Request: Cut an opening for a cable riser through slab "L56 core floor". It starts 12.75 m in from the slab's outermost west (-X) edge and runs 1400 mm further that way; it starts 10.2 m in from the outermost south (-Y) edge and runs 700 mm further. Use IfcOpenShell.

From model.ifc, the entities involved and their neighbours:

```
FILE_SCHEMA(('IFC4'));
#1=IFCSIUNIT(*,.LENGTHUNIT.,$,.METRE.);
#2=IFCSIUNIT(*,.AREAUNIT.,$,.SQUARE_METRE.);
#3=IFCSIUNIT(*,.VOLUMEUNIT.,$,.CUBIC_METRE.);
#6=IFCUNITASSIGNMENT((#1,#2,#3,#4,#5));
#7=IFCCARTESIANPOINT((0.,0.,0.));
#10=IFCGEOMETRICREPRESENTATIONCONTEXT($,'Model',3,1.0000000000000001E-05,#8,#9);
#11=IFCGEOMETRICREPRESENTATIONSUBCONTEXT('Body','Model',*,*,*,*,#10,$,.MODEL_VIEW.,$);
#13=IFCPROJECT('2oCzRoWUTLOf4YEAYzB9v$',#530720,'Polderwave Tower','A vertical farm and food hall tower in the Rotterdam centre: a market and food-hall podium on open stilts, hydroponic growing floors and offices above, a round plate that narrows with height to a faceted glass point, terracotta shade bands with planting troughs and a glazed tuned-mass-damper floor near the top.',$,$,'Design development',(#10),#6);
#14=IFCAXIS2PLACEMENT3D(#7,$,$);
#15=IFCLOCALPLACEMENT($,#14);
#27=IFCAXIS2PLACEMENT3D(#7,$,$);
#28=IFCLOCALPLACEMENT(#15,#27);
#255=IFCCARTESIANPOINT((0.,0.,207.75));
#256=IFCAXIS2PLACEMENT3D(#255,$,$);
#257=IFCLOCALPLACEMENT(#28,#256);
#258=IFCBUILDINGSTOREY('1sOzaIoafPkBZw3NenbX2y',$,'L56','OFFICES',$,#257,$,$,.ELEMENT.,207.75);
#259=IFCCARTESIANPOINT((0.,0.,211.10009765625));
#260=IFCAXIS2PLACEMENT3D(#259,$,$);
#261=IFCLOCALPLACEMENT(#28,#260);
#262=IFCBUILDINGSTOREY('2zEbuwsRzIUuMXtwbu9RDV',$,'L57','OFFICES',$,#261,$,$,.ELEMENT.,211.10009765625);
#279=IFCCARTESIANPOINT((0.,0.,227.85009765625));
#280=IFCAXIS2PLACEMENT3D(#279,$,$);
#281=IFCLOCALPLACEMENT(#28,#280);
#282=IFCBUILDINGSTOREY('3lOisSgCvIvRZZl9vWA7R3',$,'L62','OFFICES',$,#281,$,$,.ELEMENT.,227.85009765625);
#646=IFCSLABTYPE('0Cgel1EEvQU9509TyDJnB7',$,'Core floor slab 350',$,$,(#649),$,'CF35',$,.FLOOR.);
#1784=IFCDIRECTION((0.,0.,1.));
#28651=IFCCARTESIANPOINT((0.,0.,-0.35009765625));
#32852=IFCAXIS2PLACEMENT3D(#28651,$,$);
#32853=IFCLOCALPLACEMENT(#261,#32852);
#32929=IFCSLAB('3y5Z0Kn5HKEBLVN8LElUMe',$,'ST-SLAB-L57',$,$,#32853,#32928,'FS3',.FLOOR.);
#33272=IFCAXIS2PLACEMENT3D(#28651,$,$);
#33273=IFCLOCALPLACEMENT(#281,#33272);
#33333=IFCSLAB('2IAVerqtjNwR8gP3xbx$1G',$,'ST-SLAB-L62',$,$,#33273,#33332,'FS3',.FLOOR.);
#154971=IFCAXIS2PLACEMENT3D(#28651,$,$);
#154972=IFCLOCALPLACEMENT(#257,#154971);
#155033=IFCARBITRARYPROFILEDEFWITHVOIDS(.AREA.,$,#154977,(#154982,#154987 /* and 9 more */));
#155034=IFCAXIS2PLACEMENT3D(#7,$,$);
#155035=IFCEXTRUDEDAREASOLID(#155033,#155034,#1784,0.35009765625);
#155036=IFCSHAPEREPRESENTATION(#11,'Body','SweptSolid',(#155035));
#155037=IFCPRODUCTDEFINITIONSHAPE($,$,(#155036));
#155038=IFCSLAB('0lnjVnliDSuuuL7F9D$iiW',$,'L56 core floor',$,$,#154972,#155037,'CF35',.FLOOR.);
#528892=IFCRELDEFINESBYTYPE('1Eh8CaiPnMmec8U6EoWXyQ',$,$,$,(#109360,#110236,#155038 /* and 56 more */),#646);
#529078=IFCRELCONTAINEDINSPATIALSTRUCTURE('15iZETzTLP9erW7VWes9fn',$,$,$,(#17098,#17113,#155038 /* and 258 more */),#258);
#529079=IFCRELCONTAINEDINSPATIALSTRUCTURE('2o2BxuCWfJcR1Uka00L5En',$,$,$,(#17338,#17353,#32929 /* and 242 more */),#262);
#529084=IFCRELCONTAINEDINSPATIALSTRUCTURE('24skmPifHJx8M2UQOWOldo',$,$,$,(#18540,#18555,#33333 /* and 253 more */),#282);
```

```python
import numpy as np
import ifcopenshell
import ifcopenshell.api.feature
import ifcopenshell.api.geometry
import ifcopenshell.api.root
import ifcopenshell.geom
import ifcopenshell.util.placement
import ifcopenshell.util.representation
import ifcopenshell.util.shape
import ifcopenshell.util.unit

model = ifcopenshell.open("model.ifc")
unit_scale = ifcopenshell.util.unit.calculate_unit_scale(model)
settings = ifcopenshell.geom.settings()


def volume(element):
    """Net volume in cubic metres, openings subtracted."""
    shape = ifcopenshell.geom.create_shape(settings, element)
    return ifcopenshell.util.shape.get_volume(shape.geometry)


slab = model.by_guid("0lnjVnliDSuuuL7F9D$iiW")
before = volume(slab)

# Extent in the slab's own axes, in metres. The edges named are its -X and -Y sides.
slab_shape = ifcopenshell.geom.create_shape(settings, slab)
vertices = ifcopenshell.util.shape.get_vertices(slab_shape.geometry)
x_min, y_min, bottom = vertices.min(axis=0)
top = vertices[:, 2].max()

opening = ifcopenshell.api.root.create_entity(model, ifc_class="IfcOpeningElement", name="Cable riser opening", predefined_type="OPENING")
context = ifcopenshell.util.representation.get_context(model, "Model", "Body", "MODEL_VIEW")
width, depth = 1.4, 0.7
outline = [(0.0, 0.0), (width, 0.0), (width, depth), (0.0, depth), (0.0, 0.0)]
# Overshoot both faces by 50 mm so the cut is clean.
shape = ifcopenshell.api.geometry.add_slab_representation(
    model, context=context, depth=top - bottom + 0.1, polyline=outline
)
ifcopenshell.api.geometry.assign_representation(model, product=opening, representation=shape)

matrix = ifcopenshell.util.placement.get_local_placement(slab.ObjectPlacement)
matrix[:, 3] = matrix @ np.append(np.array([x_min + 12.75, y_min + 10.2, bottom - 0.05]) / unit_scale, 1.0)
ifcopenshell.api.geometry.edit_object_placement(model, product=opening, matrix=matrix, is_si=False)
ifcopenshell.api.feature.add_feature(model, feature=opening, element=slab)

after = volume(slab)

print(f"slab volume {before:.3f} -> {after:.3f} m3")

model.write("model_rev.ifc")
```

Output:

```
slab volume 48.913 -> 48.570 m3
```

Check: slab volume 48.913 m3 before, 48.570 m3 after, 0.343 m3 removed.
